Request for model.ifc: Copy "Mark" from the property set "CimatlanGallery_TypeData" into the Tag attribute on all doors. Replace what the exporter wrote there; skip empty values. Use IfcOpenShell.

First a look at what the model holds.

```python
import ifcopenshell
import ifcopenshell.util.element

model = ifcopenshell.open("model.ifc")
print(model.schema)
doors = model.by_type("IfcDoor")
print(len(doors), "doors")
for e in doors[:8]:
    source = ifcopenshell.util.element.get_pset(e, "CimatlanGallery_TypeData", "Mark")
    target = e.Tag
    print(e.id(), repr(source), repr(target), sep=" | ")
```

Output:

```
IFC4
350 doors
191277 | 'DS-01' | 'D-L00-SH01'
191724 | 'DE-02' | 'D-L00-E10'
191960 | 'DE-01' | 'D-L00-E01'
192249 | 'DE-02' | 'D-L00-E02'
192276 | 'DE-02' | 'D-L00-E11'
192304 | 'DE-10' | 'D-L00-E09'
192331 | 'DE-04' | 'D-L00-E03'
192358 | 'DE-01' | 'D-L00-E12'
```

```python
import ifcopenshell
import ifcopenshell.util.element

model = ifcopenshell.open("model.ifc")

count = 0
for e in model.by_type("IfcDoor"):
    value = ifcopenshell.util.element.get_pset(e, "CimatlanGallery_TypeData", "Mark")
    current = e.Tag
    if not value or not value.strip() or current == value:
        continue
    e.Tag = value
    count += 1

print(count, "doors updated")

model.write("model_v2.ifc")
```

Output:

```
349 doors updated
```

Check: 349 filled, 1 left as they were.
